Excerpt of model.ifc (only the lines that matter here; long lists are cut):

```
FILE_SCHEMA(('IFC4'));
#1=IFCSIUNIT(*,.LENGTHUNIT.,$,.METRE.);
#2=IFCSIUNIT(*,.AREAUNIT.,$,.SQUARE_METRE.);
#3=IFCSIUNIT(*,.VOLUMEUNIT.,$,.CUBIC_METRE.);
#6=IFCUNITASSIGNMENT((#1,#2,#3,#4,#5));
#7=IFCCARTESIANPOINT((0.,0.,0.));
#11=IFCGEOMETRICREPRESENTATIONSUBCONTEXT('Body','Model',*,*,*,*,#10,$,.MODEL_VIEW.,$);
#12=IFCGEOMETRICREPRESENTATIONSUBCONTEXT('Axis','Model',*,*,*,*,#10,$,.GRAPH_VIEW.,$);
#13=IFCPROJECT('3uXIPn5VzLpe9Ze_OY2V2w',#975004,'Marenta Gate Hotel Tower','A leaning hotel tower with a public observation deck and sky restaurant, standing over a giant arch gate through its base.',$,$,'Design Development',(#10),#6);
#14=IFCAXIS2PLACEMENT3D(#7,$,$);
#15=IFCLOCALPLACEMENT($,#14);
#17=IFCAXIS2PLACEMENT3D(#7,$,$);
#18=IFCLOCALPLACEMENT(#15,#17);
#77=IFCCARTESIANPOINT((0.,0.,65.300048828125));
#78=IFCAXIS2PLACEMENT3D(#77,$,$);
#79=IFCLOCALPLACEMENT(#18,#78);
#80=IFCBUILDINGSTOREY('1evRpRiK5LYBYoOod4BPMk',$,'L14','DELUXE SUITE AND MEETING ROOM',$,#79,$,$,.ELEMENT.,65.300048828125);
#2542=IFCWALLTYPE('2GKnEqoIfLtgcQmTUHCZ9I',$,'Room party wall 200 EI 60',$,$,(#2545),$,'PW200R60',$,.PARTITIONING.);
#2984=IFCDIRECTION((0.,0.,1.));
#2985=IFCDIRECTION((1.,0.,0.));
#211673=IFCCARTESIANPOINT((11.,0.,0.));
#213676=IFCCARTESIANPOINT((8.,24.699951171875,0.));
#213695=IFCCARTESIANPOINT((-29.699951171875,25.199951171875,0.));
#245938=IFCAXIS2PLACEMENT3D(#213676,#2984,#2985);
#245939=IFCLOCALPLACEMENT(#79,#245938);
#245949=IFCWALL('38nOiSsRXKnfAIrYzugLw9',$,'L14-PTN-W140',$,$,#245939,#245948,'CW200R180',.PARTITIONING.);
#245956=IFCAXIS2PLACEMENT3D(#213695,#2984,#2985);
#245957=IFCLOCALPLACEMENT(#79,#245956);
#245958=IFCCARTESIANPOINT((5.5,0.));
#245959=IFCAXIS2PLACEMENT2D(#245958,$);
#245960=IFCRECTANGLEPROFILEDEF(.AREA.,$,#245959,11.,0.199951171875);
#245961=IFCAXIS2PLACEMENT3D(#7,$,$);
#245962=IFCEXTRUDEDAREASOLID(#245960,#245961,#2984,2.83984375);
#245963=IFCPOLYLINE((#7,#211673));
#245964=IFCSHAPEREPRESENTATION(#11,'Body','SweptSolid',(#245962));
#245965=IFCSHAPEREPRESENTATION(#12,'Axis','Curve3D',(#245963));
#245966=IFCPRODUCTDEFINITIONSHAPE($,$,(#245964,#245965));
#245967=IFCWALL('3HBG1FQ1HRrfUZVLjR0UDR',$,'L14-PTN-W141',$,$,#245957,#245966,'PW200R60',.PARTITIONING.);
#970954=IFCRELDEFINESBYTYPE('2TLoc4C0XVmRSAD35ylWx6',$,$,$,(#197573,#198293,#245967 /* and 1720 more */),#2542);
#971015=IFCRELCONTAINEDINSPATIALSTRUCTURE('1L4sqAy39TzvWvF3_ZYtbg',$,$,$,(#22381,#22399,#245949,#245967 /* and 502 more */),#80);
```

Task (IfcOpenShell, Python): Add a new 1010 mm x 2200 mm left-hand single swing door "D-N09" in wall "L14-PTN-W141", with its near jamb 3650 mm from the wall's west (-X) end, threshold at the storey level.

```python
import numpy as np
import ifcopenshell
import ifcopenshell.api.feature
import ifcopenshell.api.geometry
import ifcopenshell.api.root
import ifcopenshell.api.spatial
import ifcopenshell.geom
import ifcopenshell.util.element
import ifcopenshell.util.placement
import ifcopenshell.util.representation
import ifcopenshell.util.shape
import ifcopenshell.util.unit

model = ifcopenshell.open("model.ifc")
unit_scale = ifcopenshell.util.unit.calculate_unit_scale(model)
settings = ifcopenshell.geom.settings()


def volume(element):
    """Net volume in cubic metres, openings subtracted."""
    shape = ifcopenshell.geom.create_shape(settings, element)
    return ifcopenshell.util.shape.get_volume(shape.geometry)


wall = model.by_id(245967)
storey = ifcopenshell.util.element.get_container(wall, ifc_class="IfcBuildingStorey")
context = ifcopenshell.util.representation.get_context(model, "Model", "Body", "MODEL_VIEW")
before = volume(wall)

width, height, from_end, sill = 1.01, 2.2, 3.65, 0.0  # metres

# The wall runs along its own X axis, and the end named is its -X end.
wall_shape = ifcopenshell.geom.create_shape(settings, wall)
x, y, z = ifcopenshell.util.shape.get_vertices(wall_shape.geometry).T
start = x.min() + from_end
face, thickness = float(y.min()), float(y.max() - y.min())
wall_matrix = ifcopenshell.util.placement.get_local_placement(wall.ObjectPlacement)
level = ifcopenshell.util.placement.get_local_placement(storey.ObjectPlacement)[2, 3]


def in_wall(x, y):
    """Placement at x, y metres in the wall's axes, at sill height."""
    matrix = wall_matrix.copy()
    matrix[:, 3] = wall_matrix @ np.array([x / unit_scale, y / unit_scale, 0.0, 1.0])
    matrix[2, 3] = level + sill / unit_scale
    return matrix


# Opening: a box that overshoots both wall faces by 50 mm.
opening = ifcopenshell.api.root.create_entity(model, ifc_class="IfcOpeningElement", predefined_type="OPENING")
box = ifcopenshell.api.geometry.add_wall_representation(
    model, context=context, length=width, height=height, thickness=thickness + 0.1
)
ifcopenshell.api.geometry.assign_representation(model, product=opening, representation=box)
ifcopenshell.api.geometry.edit_object_placement(model, product=opening, matrix=in_wall(start, face - 0.05), is_si=False)
ifcopenshell.api.feature.add_feature(model, feature=opening, element=wall)

door = ifcopenshell.api.root.create_entity(model, ifc_class="IfcDoor", name="D-N09", predefined_type="DOOR")
door.OverallWidth, door.OverallHeight = width / unit_scale, height / unit_scale
door.OperationType = "SINGLE_SWING_LEFT"
body = ifcopenshell.api.geometry.add_door_representation(
    model,
    context=context,
    overall_width=door.OverallWidth,
    overall_height=door.OverallHeight,
    operation_type="SINGLE_SWING_LEFT",
    lining_properties={"LiningDepth": thickness / unit_scale, "ThresholdDepth": thickness / unit_scale},
)
ifcopenshell.api.geometry.assign_representation(model, product=door, representation=body)
ifcopenshell.api.spatial.assign_container(model, products=[door], relating_structure=storey)
ifcopenshell.api.feature.add_filling(model, opening=opening, element=door)

# The lining spans the wall, so the door starts at the wall face.
ifcopenshell.api.geometry.edit_object_placement(model, product=door, matrix=in_wall(start, face), is_si=False)

after = volume(wall)

print(f"wall volume {before:.3f} -> {after:.3f} m3")

model.write("model_rev.ifc")
```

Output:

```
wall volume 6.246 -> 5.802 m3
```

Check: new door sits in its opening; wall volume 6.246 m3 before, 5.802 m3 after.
